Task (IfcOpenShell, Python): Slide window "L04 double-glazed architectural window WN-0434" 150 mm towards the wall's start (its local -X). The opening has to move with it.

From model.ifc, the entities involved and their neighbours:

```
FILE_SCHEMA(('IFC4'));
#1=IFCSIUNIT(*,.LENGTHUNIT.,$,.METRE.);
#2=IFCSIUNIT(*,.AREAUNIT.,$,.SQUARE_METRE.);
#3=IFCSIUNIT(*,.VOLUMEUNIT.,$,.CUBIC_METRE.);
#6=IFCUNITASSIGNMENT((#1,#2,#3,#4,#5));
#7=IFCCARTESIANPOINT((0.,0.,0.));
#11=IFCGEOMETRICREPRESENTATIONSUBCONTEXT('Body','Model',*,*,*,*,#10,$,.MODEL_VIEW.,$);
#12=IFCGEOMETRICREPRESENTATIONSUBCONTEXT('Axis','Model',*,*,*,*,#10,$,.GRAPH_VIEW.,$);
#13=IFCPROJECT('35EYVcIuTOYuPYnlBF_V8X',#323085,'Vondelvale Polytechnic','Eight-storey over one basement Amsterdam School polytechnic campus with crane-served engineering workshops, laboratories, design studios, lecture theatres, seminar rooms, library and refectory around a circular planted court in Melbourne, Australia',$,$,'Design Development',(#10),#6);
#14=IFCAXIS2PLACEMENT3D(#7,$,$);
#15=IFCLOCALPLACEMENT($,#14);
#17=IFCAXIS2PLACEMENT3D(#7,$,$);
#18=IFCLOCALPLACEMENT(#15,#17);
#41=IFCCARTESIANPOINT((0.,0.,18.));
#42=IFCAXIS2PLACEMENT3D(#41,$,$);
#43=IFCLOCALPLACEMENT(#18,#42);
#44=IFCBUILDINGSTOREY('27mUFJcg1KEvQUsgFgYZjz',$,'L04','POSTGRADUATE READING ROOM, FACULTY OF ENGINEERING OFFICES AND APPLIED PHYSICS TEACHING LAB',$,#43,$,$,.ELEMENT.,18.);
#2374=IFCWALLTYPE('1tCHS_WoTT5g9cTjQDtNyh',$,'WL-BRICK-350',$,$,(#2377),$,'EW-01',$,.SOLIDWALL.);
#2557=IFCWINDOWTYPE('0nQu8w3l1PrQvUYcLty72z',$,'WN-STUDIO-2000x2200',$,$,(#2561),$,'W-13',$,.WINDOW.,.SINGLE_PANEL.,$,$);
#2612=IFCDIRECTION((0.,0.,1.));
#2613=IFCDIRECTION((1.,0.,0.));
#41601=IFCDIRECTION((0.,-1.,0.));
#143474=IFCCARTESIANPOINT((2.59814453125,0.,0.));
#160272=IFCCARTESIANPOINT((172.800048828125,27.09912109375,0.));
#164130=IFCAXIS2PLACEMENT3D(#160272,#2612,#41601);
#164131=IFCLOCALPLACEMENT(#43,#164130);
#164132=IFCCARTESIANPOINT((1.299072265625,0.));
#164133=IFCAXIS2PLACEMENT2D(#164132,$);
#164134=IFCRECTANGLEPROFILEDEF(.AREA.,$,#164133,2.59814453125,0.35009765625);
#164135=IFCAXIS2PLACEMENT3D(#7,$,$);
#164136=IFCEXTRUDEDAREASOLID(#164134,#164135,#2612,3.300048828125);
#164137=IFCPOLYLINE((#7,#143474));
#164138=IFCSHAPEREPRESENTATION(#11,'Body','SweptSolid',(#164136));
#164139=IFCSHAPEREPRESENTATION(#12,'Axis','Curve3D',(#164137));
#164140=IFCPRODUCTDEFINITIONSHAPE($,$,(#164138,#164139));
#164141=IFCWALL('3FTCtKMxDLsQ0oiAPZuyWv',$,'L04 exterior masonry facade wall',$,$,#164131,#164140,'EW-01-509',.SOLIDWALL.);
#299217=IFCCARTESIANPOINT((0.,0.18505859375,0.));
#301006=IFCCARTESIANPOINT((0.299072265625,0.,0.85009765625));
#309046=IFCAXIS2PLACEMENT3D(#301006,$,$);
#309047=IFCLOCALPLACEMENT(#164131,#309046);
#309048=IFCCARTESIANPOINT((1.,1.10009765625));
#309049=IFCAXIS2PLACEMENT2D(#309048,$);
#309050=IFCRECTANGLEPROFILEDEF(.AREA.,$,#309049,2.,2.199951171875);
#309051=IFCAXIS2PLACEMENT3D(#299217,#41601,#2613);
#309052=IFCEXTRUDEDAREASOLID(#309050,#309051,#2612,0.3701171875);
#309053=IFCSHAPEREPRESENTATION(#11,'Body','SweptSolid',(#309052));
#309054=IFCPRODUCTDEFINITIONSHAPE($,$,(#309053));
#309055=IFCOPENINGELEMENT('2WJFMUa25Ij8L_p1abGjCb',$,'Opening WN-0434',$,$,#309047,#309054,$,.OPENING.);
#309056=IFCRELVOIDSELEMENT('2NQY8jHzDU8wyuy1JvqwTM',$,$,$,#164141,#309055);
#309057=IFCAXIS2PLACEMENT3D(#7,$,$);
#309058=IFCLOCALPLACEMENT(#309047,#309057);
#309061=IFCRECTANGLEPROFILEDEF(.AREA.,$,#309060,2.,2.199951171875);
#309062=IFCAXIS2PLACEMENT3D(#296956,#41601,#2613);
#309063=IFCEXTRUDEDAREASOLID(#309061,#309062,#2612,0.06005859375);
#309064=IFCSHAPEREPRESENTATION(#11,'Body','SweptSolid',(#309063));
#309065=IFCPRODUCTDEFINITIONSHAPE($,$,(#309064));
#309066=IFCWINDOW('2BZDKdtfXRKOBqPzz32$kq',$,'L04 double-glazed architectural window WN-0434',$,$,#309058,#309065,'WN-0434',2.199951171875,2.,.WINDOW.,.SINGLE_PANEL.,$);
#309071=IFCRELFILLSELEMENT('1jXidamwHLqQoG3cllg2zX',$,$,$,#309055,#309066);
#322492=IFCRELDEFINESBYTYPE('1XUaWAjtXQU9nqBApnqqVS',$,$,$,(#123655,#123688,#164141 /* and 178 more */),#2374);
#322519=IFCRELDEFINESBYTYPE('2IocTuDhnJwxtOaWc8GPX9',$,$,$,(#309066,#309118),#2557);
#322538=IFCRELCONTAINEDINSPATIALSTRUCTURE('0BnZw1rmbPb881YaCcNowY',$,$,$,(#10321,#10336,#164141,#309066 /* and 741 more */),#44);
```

```python
import ifcopenshell
import ifcopenshell.api.geometry
import ifcopenshell.util.placement
import ifcopenshell.util.unit

model = ifcopenshell.open("model.ifc")
unit_scale = ifcopenshell.util.unit.calculate_unit_scale(model)

window = model.by_id(309066)
opening = window.FillsVoids[0].RelatingOpeningElement
wall = opening.VoidsElements[0].RelatingBuildingElement

wall_matrix = ifcopenshell.util.placement.get_local_placement(wall.ObjectPlacement)
shift = wall_matrix[:3, 0] * -0.15 / unit_scale
before = ifcopenshell.util.placement.get_local_placement(window.ObjectPlacement)[:3, 3].copy()

# The window is placed relative to its opening, so it follows when the opening moves.
matrix = ifcopenshell.util.placement.get_local_placement(opening.ObjectPlacement)
matrix[:3, 3] += shift
ifcopenshell.api.geometry.edit_object_placement(
    model, product=opening, matrix=matrix, is_si=False, should_transform_children=True
)

after = ifcopenshell.util.placement.get_local_placement(window.ObjectPlacement)[:3, 3]
print("window moved by", (after - before).round(3) + 0.0)

model.write("model_updated.ifc")
```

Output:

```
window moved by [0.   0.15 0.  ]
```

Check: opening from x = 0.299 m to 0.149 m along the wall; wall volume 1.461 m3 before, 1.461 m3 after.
